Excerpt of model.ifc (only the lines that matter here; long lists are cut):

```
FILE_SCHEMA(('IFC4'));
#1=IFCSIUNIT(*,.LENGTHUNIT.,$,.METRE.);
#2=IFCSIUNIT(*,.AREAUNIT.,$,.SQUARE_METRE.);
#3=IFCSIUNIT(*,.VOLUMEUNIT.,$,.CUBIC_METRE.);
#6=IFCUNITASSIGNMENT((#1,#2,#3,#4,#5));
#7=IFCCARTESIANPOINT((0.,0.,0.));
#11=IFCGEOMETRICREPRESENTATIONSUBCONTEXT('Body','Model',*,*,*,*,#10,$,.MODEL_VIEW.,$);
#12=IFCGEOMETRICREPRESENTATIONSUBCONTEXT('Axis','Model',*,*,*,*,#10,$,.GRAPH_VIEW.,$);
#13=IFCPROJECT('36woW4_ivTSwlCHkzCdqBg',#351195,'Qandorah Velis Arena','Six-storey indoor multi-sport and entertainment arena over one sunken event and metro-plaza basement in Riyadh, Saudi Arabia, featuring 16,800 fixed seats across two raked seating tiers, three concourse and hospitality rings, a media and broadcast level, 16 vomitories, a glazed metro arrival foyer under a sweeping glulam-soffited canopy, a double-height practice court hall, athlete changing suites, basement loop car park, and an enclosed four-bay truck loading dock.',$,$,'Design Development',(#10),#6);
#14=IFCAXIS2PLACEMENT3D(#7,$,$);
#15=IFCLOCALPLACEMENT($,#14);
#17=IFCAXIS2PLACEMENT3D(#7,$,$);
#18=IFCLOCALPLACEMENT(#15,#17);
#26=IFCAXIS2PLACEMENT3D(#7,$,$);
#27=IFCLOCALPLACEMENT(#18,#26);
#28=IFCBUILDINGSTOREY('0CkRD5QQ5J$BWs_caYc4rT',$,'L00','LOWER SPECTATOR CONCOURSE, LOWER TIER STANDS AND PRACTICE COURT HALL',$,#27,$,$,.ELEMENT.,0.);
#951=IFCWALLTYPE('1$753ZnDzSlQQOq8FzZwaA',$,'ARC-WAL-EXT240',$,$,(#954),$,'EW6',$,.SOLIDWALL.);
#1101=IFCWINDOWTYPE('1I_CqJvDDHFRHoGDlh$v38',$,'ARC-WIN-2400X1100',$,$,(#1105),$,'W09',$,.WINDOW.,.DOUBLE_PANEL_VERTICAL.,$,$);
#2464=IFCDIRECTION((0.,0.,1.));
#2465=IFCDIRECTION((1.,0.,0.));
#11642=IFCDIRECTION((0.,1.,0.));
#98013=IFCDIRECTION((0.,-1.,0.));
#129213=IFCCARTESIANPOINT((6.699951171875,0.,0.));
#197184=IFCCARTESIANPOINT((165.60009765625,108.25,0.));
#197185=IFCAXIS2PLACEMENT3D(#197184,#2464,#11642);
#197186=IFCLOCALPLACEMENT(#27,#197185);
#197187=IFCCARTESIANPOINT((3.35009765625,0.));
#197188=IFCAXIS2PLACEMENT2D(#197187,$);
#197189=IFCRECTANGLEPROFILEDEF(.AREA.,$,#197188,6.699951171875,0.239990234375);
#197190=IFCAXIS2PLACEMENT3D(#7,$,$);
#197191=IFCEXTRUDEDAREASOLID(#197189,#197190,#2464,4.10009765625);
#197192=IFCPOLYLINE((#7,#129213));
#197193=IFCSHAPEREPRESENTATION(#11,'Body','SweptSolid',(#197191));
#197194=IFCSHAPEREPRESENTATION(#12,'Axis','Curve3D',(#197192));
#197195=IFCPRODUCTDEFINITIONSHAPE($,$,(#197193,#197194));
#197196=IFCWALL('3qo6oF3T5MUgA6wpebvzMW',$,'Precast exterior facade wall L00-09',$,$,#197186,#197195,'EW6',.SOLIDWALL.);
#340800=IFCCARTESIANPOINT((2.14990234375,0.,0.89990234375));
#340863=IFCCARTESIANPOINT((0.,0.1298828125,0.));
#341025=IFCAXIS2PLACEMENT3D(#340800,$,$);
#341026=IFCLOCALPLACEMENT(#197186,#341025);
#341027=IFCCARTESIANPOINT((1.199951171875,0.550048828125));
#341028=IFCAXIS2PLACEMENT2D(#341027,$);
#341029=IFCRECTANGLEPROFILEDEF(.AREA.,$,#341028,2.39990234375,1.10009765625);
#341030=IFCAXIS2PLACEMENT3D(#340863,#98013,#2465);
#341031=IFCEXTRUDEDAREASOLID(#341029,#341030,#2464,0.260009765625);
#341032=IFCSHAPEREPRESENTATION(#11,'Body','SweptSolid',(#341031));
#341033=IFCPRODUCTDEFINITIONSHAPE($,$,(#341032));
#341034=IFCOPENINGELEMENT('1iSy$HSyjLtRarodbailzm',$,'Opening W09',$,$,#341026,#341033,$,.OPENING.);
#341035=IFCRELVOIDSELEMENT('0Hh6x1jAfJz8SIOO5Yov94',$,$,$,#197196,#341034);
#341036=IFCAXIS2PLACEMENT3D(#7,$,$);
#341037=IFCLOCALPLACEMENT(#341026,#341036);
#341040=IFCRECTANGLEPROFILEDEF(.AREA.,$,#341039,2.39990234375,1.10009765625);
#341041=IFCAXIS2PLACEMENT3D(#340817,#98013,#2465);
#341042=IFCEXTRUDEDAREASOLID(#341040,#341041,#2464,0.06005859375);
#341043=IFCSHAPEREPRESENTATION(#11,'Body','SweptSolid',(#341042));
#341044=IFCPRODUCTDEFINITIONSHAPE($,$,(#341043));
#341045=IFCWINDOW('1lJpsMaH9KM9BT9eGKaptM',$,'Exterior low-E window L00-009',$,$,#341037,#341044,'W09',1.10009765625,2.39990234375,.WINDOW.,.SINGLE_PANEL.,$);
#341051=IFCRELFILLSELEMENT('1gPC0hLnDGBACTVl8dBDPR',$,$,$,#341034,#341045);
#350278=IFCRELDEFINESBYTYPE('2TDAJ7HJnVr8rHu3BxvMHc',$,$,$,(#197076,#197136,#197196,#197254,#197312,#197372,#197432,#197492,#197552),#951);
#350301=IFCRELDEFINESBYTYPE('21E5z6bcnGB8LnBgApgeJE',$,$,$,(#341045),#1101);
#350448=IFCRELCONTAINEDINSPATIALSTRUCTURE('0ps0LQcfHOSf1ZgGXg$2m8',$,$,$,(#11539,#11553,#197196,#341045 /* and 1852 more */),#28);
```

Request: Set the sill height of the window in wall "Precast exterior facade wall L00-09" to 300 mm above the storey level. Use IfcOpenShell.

```python
import numpy as np
import ifcopenshell
import ifcopenshell.api.geometry
import ifcopenshell.geom
import ifcopenshell.util.element
import ifcopenshell.util.placement
import ifcopenshell.util.shape
import ifcopenshell.util.unit

model = ifcopenshell.open("model.ifc")
unit_scale = ifcopenshell.util.unit.calculate_unit_scale(model)

window = model.by_guid("1lJpsMaH9KM9BT9eGKaptM")
opening = window.FillsVoids[0].RelatingOpeningElement
storey = ifcopenshell.util.element.get_container(window, ifc_class="IfcBuildingStorey")
level = ifcopenshell.util.placement.get_local_placement(storey.ObjectPlacement)[2, 3]

# The opening's origin need not be at the sill, so measure its lowest point.
shape = ifcopenshell.geom.create_shape(ifcopenshell.geom.settings(), opening)
bottom = ifcopenshell.util.shape.get_shape_bottom_elevation(shape, shape.geometry) / unit_scale
dz = level + 0.3 - bottom

shift = np.array([0.0, 0.0, dz])
# The window is placed relative to its opening, so it follows when the opening moves.
matrix = ifcopenshell.util.placement.get_local_placement(opening.ObjectPlacement)
matrix[:3, 3] += shift
ifcopenshell.api.geometry.edit_object_placement(
    model, product=opening, matrix=matrix, is_si=False, should_transform_children=True
)

print(f"moved by {dz * unit_scale:+.3f} m")

model.write("model_edited.ifc")
```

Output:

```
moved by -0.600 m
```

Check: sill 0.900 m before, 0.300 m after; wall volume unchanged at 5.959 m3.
